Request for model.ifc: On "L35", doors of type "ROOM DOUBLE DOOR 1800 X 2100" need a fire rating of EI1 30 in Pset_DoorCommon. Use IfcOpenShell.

First a look at what the model holds.

```python
import ifcopenshell
import ifcopenshell.util.element

model = ifcopenshell.open("model.ifc")
print(model.schema)
storey = next(s for s in model.by_type("IfcBuildingStorey") if s.Name == "L35")
doors = [e for e in ifcopenshell.util.element.get_decomposition(storey) if e.is_a("IfcDoor")]
seen = {}
for e in doors:
    element_type = ifcopenshell.util.element.get_type(e)
    key = (element_type.Name if element_type != e and element_type else None, ifcopenshell.util.element.get_pset(e, "Pset_DoorCommon", "FireRating"))
    seen[key] = seen.get(key, 0) + 1
for (name, value), count in sorted(seen.items(), key=str):
    print(count, "x", name, "|", value)
```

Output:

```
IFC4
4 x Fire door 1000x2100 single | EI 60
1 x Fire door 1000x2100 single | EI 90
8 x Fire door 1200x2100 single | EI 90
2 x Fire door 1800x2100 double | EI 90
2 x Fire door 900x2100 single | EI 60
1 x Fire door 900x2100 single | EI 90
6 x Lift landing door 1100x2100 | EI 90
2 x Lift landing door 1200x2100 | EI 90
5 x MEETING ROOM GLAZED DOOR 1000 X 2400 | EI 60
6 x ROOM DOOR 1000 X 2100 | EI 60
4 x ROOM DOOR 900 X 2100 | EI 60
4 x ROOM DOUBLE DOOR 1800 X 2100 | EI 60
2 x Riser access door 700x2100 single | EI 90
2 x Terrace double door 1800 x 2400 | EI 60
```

```python
import ifcopenshell
import ifcopenshell.api.pset
import ifcopenshell.util.element

model = ifcopenshell.open("model.ifc")

storey = next(s for s in model.by_type("IfcBuildingStorey") if s.Name == "L35")
doors = [e for e in ifcopenshell.util.element.get_decomposition(storey) if e.is_a("IfcDoor")]

count = 0
for e in doors:
    element_type = ifcopenshell.util.element.get_type(e)
    if element_type in (None, e) or element_type.Name != "ROOM DOUBLE DOOR 1800 X 2100":
        continue
    # add_pset returns the element's existing set when there is one.
    pset = ifcopenshell.api.pset.add_pset(model, product=e, name="Pset_DoorCommon")
    ifcopenshell.api.pset.edit_pset(model, pset=pset, properties={"FireRating": "EI1 30"})
    count += 1

print(count, "doors updated")

model.write("model-out.ifc")
```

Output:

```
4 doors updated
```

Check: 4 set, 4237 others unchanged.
